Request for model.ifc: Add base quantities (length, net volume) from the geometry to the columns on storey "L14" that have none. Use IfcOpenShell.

First a look at what the model holds.

```python
import ifcopenshell
import ifcopenshell.util.element
import ifcopenshell.util.unit

model = ifcopenshell.open("model.ifc")
print(model.schema)
for unit_type in ("LENGTHUNIT", "AREAUNIT", "VOLUMEUNIT"):
    print(unit_type, ifcopenshell.util.unit.calculate_unit_scale(model, unit_type))
storey = next(s for s in model.by_type("IfcBuildingStorey") if s.Name == "L14")
columns = [e for e in ifcopenshell.util.element.get_decomposition(storey) if e.is_a("IfcColumn")]
for e in sorted(columns, key=lambda e: e.id()):
    print(e.id(), e.is_a(), e.Name, list(ifcopenshell.util.element.get_psets(e, qtos_only=True)), sep=" | ")
```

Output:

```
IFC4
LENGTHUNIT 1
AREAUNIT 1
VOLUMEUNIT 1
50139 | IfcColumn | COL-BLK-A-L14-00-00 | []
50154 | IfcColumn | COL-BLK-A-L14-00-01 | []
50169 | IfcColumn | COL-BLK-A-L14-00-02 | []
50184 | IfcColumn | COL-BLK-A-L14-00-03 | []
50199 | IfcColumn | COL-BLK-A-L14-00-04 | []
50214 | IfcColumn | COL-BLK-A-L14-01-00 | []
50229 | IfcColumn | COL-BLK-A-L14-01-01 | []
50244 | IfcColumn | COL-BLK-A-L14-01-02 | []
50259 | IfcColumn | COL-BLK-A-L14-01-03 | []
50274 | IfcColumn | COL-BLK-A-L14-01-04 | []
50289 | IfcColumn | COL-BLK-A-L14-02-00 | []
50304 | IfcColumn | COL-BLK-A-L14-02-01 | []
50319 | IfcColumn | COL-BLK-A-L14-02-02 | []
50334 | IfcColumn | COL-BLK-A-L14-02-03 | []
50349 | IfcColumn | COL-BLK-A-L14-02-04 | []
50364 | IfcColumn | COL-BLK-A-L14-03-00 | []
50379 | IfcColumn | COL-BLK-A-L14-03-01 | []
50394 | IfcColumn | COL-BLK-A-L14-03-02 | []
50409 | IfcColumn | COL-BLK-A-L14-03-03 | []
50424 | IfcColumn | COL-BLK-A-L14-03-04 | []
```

```python
import ifcopenshell
import ifcopenshell.api.pset
import ifcopenshell.geom
import ifcopenshell.util.element
import ifcopenshell.util.shape
import ifcopenshell.util.unit

model = ifcopenshell.open("model.ifc")
unit_scale = ifcopenshell.util.unit.calculate_unit_scale(model)
volume_scale = ifcopenshell.util.unit.calculate_unit_scale(model, "VOLUMEUNIT")
settings = ifcopenshell.geom.settings()

storey = next(s for s in model.by_type("IfcBuildingStorey") if s.Name == "L14")
columns = [e for e in ifcopenshell.util.element.get_decomposition(storey) if e.is_a("IfcColumn")]

for e in sorted(columns, key=lambda e: e.id()):
    if ifcopenshell.util.element.get_psets(e, qtos_only=True, should_inherit=False):
        continue
    # Geometry comes back in metres, in the element's own axes.
    shape = ifcopenshell.geom.create_shape(settings, e)
    values = {
        "Length": ifcopenshell.util.shape.get_z(shape.geometry) / unit_scale,
        "NetVolume": ifcopenshell.util.shape.get_volume(shape.geometry) / volume_scale,
    }
    qto = ifcopenshell.api.pset.add_qto(model, product=e, name="Qto_ColumnBaseQuantities")
    ifcopenshell.api.pset.edit_qto(model, qto=qto, properties=values)
    print(e.id(), {k: round(v, 3) for k, v in values.items()})

model.write("model_edited.ifc")
```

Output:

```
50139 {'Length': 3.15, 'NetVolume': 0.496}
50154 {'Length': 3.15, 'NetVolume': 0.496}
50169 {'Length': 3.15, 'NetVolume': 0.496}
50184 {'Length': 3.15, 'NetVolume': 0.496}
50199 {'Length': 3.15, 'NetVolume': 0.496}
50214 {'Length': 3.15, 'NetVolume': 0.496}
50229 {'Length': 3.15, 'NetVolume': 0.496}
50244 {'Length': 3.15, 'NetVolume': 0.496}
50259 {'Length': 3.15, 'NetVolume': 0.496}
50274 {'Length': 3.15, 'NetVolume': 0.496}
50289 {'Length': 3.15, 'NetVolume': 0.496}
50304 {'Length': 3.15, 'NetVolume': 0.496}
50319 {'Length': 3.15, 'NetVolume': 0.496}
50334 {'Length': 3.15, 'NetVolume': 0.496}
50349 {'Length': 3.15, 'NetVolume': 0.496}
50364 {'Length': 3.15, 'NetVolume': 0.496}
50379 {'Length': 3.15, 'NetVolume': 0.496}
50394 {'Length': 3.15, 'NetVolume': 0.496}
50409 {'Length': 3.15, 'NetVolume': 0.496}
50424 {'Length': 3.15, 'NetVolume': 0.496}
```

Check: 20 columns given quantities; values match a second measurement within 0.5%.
